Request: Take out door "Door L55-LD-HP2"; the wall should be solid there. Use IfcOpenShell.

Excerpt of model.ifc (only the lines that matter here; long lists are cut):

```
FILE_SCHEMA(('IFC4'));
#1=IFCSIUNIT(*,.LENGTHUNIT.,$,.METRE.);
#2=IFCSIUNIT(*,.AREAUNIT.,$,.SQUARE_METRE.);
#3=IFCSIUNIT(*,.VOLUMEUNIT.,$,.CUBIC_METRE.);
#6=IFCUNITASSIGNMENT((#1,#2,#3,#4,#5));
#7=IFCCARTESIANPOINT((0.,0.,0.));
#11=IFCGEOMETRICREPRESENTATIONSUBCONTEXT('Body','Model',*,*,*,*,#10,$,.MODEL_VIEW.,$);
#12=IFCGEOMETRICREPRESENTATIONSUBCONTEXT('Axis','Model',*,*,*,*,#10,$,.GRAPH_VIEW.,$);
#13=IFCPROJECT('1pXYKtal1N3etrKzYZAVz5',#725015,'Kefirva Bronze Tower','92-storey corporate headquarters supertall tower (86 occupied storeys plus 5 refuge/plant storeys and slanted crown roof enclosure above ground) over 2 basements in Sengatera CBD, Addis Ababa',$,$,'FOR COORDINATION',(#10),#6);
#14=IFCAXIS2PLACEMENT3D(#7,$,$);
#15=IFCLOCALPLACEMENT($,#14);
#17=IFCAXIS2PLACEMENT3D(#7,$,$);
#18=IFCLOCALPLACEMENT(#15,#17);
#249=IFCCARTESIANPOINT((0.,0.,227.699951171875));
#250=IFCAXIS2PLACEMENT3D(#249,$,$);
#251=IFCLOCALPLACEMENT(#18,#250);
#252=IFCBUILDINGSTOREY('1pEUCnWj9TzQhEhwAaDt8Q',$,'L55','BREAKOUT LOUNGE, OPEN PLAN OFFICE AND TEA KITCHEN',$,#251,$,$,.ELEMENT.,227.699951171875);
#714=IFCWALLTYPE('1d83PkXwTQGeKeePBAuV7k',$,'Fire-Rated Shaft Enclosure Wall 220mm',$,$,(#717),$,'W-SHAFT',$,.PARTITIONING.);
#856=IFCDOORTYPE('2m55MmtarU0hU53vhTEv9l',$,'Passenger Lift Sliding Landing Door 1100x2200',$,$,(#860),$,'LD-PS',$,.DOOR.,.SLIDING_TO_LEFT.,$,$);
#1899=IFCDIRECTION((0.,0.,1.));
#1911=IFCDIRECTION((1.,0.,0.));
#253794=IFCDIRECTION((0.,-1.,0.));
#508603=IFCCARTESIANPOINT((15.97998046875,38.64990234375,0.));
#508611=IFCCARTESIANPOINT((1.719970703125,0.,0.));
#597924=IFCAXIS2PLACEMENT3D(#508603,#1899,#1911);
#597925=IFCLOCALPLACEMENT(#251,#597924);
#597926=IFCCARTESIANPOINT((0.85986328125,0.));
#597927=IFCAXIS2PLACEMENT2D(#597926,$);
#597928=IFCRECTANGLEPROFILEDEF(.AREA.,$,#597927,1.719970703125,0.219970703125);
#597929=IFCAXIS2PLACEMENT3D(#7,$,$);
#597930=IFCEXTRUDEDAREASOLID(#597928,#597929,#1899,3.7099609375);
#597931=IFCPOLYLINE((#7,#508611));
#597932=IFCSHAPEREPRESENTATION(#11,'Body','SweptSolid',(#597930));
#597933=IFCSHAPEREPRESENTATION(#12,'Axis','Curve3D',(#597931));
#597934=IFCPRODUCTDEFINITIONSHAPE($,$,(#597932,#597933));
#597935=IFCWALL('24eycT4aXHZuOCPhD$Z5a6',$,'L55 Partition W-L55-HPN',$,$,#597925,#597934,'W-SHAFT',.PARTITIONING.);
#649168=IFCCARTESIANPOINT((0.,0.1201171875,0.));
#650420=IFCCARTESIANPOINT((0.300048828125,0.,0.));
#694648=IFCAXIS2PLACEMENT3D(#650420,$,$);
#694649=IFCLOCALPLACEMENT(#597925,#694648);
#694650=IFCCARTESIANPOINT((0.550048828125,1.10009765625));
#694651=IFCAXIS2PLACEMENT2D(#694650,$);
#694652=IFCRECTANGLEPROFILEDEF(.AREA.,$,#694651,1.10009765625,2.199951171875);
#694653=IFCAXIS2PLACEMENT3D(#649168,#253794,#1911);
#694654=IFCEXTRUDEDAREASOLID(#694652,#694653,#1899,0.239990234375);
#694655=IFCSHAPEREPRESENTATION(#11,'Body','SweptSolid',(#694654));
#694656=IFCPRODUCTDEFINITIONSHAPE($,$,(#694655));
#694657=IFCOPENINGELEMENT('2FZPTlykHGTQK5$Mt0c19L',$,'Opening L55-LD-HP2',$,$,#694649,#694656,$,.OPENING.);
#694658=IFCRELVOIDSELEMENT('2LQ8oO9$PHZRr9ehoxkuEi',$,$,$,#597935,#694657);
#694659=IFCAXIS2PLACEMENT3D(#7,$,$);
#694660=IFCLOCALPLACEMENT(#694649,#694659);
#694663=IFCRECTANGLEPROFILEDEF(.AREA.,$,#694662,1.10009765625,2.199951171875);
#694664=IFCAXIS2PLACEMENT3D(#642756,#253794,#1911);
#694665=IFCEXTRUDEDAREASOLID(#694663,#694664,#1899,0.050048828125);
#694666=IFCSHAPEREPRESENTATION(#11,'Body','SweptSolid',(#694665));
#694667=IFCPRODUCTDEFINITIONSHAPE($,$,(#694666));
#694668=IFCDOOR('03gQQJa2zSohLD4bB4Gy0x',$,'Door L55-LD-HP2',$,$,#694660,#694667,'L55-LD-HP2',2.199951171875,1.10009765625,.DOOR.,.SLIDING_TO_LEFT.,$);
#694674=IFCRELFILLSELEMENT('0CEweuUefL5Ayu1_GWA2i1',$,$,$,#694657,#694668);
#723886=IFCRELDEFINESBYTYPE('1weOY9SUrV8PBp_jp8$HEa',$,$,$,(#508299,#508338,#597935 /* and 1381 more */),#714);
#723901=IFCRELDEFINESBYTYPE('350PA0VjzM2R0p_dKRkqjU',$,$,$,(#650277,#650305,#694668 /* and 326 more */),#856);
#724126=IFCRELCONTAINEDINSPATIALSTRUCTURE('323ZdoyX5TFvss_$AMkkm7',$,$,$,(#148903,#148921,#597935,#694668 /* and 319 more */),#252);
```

```python
import ifcopenshell
import ifcopenshell.api.feature
import ifcopenshell.api.root
import ifcopenshell.geom
import ifcopenshell.util.shape

model = ifcopenshell.open("model.ifc")
settings = ifcopenshell.geom.settings()


def volume(element):
    """Net volume in cubic metres, openings subtracted."""
    shape = ifcopenshell.geom.create_shape(settings, element)
    return ifcopenshell.util.shape.get_volume(shape.geometry)


door = model.by_guid("03gQQJa2zSohLD4bB4Gy0x")
opening = door.FillsVoids[0].RelatingOpeningElement
wall = opening.VoidsElements[0].RelatingBuildingElement
before = volume(wall)

ifcopenshell.api.root.remove_product(model, product=door)
ifcopenshell.api.feature.remove_feature(model, feature=opening)

after = volume(wall)

print(f"wall volume {before:.3f} -> {after:.3f} m3")

model.write("model-out.ifc")
```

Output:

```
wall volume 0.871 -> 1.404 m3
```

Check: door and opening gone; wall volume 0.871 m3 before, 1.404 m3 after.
